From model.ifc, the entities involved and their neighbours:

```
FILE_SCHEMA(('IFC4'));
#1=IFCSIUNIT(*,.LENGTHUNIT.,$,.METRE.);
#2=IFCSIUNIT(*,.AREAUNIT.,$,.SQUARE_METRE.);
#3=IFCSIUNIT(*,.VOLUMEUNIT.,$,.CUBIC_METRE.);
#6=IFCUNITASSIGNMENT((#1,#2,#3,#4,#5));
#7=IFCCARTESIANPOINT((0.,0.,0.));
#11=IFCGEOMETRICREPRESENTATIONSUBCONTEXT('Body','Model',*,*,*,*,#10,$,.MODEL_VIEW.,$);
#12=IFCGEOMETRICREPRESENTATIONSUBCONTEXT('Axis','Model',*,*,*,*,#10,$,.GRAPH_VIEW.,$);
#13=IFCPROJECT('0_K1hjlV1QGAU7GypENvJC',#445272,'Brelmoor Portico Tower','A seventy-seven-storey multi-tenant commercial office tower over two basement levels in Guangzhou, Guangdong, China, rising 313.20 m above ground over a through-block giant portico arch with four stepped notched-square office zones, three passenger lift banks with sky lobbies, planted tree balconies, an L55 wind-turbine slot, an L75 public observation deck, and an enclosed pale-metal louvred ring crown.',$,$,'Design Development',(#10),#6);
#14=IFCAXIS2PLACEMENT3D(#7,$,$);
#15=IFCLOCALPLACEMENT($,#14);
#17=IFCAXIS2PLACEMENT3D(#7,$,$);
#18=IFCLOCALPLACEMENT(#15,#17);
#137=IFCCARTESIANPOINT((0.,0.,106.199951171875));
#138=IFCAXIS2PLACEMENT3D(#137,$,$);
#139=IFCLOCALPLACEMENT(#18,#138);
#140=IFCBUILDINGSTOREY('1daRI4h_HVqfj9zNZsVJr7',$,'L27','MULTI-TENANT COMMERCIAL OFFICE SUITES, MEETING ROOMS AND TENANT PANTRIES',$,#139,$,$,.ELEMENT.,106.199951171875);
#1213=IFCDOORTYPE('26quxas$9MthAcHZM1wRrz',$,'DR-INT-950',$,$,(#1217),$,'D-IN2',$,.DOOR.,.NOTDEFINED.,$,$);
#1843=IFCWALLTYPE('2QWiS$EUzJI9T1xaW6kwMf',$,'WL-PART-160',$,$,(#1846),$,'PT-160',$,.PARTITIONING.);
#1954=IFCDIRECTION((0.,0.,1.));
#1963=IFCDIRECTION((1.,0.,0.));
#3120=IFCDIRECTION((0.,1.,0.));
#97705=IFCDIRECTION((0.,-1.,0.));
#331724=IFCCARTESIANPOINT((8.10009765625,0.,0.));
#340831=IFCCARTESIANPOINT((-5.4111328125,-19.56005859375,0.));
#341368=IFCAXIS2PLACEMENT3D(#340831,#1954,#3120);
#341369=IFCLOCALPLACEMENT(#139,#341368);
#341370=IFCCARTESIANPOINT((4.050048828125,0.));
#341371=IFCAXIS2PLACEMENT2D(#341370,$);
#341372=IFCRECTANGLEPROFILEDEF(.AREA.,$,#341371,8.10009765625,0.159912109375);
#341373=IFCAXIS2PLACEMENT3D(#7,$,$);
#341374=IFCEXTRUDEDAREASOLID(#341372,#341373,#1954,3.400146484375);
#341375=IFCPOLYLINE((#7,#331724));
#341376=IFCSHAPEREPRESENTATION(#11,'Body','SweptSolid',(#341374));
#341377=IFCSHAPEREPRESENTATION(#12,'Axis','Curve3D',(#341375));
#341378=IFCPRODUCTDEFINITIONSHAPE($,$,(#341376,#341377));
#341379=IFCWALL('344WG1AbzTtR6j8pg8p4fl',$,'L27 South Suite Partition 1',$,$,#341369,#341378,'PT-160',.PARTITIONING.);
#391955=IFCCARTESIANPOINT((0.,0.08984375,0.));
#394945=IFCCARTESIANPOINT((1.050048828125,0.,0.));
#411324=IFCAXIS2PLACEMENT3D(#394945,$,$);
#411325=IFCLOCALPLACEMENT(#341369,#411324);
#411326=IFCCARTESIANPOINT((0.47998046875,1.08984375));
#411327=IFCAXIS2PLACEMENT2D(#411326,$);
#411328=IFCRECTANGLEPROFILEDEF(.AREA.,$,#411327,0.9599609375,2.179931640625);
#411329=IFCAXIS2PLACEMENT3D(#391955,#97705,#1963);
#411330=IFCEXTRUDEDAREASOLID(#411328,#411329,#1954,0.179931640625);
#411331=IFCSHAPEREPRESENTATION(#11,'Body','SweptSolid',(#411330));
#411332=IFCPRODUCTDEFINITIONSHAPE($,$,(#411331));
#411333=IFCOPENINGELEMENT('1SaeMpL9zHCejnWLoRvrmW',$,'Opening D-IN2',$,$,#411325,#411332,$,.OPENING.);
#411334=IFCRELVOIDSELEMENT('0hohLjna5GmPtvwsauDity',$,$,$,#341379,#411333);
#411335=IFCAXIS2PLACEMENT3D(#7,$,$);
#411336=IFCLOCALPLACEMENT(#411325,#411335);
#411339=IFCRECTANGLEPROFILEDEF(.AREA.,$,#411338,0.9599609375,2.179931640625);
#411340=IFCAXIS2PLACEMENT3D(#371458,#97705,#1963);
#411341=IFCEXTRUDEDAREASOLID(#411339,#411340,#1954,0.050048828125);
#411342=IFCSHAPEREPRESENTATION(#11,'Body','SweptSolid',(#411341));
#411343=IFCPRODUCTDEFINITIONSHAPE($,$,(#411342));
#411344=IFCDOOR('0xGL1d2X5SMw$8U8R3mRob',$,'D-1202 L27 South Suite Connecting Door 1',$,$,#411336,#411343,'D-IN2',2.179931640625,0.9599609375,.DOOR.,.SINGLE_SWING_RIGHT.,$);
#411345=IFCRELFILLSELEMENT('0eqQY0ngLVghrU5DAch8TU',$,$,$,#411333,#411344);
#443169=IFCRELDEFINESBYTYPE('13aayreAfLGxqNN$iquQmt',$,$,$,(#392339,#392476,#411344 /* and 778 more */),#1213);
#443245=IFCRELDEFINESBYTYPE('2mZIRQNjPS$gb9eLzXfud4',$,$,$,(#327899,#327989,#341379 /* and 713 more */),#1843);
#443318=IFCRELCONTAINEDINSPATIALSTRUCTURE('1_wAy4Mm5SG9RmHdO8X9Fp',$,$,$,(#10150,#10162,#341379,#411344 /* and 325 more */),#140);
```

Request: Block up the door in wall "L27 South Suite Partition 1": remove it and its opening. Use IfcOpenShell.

```python
import ifcopenshell
import ifcopenshell.api.feature
import ifcopenshell.api.root
import ifcopenshell.geom
import ifcopenshell.util.shape

model = ifcopenshell.open("model.ifc")
settings = ifcopenshell.geom.settings()


def volume(element):
    """Net volume in cubic metres, openings subtracted."""
    shape = ifcopenshell.geom.create_shape(settings, element)
    return ifcopenshell.util.shape.get_volume(shape.geometry)


door = model.by_guid("0xGL1d2X5SMw$8U8R3mRob")
opening = door.FillsVoids[0].RelatingOpeningElement
wall = opening.VoidsElements[0].RelatingBuildingElement
before = volume(wall)

ifcopenshell.api.root.remove_product(model, product=door)
ifcopenshell.api.feature.remove_feature(model, feature=opening)

after = volume(wall)

print(f"wall volume {before:.3f} -> {after:.3f} m3")

model.write("model_rev.ifc")
```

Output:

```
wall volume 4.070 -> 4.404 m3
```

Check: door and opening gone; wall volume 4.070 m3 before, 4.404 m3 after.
